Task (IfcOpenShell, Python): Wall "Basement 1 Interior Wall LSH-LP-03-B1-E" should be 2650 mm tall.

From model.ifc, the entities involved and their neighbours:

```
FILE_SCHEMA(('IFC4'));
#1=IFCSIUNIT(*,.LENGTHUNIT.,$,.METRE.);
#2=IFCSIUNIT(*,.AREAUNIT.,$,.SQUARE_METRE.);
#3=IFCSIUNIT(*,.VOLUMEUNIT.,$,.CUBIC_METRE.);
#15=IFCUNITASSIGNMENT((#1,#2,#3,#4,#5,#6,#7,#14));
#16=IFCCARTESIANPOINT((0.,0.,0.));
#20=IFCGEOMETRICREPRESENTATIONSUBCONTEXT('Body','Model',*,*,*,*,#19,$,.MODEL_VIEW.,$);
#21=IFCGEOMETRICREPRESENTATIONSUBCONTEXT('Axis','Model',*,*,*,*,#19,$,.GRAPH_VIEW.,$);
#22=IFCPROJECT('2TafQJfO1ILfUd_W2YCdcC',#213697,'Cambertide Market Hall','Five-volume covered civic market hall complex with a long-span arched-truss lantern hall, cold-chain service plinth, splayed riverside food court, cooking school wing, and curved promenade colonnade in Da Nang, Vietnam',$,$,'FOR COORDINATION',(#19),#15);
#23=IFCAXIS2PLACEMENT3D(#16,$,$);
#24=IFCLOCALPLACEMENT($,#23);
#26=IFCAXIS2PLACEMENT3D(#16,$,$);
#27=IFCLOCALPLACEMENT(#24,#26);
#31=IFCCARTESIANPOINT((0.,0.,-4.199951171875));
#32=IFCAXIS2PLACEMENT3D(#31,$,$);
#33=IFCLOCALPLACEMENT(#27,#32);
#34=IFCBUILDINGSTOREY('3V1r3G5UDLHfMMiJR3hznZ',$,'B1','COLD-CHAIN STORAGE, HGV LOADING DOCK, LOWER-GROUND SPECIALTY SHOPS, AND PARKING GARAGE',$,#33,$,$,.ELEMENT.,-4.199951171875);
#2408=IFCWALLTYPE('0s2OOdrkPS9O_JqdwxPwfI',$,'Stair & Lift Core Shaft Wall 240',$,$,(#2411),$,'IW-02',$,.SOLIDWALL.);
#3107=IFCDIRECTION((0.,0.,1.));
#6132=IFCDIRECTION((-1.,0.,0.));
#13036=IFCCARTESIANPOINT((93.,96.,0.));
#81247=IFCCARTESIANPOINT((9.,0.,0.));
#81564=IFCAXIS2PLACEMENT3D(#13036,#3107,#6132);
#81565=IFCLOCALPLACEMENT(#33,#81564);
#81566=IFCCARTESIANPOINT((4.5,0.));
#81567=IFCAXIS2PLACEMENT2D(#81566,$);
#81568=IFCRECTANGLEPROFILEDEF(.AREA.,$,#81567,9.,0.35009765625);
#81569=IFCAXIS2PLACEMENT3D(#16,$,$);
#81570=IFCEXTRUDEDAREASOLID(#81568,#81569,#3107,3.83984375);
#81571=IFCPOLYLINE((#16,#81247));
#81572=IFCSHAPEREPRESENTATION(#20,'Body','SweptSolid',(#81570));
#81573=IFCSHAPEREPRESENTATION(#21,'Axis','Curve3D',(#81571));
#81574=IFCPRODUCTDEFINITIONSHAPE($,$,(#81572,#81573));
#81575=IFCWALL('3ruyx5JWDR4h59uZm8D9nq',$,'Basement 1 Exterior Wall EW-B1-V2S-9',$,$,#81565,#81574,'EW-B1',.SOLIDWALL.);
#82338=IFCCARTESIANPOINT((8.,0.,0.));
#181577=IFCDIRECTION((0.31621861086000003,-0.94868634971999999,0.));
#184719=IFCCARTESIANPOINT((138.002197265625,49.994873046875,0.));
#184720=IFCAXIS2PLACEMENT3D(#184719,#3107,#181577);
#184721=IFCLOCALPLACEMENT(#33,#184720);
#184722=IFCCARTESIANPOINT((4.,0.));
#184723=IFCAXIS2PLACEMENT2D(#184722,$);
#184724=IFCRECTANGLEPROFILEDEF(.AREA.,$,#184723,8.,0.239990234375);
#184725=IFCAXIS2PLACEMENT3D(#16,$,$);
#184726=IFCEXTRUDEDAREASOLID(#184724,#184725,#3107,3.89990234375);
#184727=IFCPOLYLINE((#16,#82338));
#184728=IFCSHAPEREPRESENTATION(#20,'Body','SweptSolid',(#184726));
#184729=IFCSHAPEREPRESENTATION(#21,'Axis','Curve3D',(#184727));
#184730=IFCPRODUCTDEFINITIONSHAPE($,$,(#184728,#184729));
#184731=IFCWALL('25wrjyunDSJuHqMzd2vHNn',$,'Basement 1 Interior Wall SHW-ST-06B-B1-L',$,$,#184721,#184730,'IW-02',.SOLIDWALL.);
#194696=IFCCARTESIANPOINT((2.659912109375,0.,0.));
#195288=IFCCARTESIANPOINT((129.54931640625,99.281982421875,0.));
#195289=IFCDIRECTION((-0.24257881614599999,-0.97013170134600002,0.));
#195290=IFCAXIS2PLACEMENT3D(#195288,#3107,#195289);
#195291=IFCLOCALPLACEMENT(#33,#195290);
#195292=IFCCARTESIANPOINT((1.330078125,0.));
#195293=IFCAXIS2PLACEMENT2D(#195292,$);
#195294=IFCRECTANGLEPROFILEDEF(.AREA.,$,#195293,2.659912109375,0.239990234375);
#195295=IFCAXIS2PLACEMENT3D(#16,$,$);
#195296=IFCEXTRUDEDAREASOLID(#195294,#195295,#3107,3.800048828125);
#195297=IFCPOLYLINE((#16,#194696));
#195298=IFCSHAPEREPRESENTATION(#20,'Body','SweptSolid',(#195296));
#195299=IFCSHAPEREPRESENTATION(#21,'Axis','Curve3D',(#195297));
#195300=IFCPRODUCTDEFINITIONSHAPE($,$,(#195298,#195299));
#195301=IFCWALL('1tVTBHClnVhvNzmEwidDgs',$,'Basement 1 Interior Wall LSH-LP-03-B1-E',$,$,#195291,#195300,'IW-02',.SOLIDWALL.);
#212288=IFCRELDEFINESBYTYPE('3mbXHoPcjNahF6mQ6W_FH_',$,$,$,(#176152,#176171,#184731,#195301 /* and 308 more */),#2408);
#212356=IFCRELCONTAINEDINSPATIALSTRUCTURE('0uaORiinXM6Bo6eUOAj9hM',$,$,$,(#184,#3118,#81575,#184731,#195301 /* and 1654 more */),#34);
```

```python
import ifcopenshell
import ifcopenshell.geom
import ifcopenshell.util.representation
import ifcopenshell.util.shape

model = ifcopenshell.open("model.ifc")
settings = ifcopenshell.geom.settings()


def volume(element):
    """Net volume in cubic metres, openings subtracted."""
    shape = ifcopenshell.geom.create_shape(settings, element)
    return ifcopenshell.util.shape.get_volume(shape.geometry)


wall = model.by_id(195301)
before = volume(wall)

body = ifcopenshell.util.representation.get_representation(wall, "Model", "Body")
solid = body.Items[0]
old_height = solid.Depth
solid.Depth = 2.65
after = volume(wall)

print(f"height {old_height:g} -> {solid.Depth:g}, volume {before:.3f} -> {after:.3f} m3")

model.write("model_edited.ifc")
```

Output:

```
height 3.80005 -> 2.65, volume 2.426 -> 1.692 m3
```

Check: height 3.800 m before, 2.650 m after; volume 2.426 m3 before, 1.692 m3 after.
